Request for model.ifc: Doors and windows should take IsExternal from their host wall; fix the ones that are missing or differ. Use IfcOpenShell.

First a look at what the model holds.

```python
import ifcopenshell
import ifcopenshell.util.element

model = ifcopenshell.open("model.ifc")
print(model.schema)
seen = {}
for e in model.by_type("IfcDoor") + model.by_type("IfcWindow"):
    if not e.FillsVoids:
        continue
    host = e.FillsVoids[0].RelatingOpeningElement.VoidsElements[0].RelatingBuildingElement
    own = ifcopenshell.util.element.get_pset(e, f"Pset_{e.is_a()[3:].removesuffix('StandardCase')}Common", "IsExternal")
    wall = ifcopenshell.util.element.get_pset(host, "Pset_WallCommon", "IsExternal")
    seen[e.is_a(), own, wall] = seen.get((e.is_a(), own, wall), 0) + 1
for (cls, own, wall), count in sorted(seen.items(), key=str):
    print(count, cls, "IsExternal:", own, "| host wall:", wall)
```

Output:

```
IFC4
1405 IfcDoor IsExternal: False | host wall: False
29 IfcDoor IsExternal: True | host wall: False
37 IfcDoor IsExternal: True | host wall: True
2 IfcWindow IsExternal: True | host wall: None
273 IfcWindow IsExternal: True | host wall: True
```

```python
import ifcopenshell
import ifcopenshell.api.pset
import ifcopenshell.util.element

model = ifcopenshell.open("model.ifc")

count = 0
for ifc_class, pset_name in (("IfcDoor", "Pset_DoorCommon"), ("IfcWindow", "Pset_WindowCommon")):
    for e in model.by_type(ifc_class):
        if not e.FillsVoids:
            continue
        host = e.FillsVoids[0].RelatingOpeningElement.VoidsElements[0].RelatingBuildingElement
        external = ifcopenshell.util.element.get_pset(host, "Pset_WallCommon", "IsExternal")
        if external is None or ifcopenshell.util.element.get_pset(e, pset_name, "IsExternal") == external:
            continue
        pset = ifcopenshell.api.pset.add_pset(model, product=e, name=pset_name)
        ifcopenshell.api.pset.edit_pset(model, pset=pset, properties={"IsExternal": external})
        count += 1

print(count, "updated")

model.write("model_updated.ifc")
```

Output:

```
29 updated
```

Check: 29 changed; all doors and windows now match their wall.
